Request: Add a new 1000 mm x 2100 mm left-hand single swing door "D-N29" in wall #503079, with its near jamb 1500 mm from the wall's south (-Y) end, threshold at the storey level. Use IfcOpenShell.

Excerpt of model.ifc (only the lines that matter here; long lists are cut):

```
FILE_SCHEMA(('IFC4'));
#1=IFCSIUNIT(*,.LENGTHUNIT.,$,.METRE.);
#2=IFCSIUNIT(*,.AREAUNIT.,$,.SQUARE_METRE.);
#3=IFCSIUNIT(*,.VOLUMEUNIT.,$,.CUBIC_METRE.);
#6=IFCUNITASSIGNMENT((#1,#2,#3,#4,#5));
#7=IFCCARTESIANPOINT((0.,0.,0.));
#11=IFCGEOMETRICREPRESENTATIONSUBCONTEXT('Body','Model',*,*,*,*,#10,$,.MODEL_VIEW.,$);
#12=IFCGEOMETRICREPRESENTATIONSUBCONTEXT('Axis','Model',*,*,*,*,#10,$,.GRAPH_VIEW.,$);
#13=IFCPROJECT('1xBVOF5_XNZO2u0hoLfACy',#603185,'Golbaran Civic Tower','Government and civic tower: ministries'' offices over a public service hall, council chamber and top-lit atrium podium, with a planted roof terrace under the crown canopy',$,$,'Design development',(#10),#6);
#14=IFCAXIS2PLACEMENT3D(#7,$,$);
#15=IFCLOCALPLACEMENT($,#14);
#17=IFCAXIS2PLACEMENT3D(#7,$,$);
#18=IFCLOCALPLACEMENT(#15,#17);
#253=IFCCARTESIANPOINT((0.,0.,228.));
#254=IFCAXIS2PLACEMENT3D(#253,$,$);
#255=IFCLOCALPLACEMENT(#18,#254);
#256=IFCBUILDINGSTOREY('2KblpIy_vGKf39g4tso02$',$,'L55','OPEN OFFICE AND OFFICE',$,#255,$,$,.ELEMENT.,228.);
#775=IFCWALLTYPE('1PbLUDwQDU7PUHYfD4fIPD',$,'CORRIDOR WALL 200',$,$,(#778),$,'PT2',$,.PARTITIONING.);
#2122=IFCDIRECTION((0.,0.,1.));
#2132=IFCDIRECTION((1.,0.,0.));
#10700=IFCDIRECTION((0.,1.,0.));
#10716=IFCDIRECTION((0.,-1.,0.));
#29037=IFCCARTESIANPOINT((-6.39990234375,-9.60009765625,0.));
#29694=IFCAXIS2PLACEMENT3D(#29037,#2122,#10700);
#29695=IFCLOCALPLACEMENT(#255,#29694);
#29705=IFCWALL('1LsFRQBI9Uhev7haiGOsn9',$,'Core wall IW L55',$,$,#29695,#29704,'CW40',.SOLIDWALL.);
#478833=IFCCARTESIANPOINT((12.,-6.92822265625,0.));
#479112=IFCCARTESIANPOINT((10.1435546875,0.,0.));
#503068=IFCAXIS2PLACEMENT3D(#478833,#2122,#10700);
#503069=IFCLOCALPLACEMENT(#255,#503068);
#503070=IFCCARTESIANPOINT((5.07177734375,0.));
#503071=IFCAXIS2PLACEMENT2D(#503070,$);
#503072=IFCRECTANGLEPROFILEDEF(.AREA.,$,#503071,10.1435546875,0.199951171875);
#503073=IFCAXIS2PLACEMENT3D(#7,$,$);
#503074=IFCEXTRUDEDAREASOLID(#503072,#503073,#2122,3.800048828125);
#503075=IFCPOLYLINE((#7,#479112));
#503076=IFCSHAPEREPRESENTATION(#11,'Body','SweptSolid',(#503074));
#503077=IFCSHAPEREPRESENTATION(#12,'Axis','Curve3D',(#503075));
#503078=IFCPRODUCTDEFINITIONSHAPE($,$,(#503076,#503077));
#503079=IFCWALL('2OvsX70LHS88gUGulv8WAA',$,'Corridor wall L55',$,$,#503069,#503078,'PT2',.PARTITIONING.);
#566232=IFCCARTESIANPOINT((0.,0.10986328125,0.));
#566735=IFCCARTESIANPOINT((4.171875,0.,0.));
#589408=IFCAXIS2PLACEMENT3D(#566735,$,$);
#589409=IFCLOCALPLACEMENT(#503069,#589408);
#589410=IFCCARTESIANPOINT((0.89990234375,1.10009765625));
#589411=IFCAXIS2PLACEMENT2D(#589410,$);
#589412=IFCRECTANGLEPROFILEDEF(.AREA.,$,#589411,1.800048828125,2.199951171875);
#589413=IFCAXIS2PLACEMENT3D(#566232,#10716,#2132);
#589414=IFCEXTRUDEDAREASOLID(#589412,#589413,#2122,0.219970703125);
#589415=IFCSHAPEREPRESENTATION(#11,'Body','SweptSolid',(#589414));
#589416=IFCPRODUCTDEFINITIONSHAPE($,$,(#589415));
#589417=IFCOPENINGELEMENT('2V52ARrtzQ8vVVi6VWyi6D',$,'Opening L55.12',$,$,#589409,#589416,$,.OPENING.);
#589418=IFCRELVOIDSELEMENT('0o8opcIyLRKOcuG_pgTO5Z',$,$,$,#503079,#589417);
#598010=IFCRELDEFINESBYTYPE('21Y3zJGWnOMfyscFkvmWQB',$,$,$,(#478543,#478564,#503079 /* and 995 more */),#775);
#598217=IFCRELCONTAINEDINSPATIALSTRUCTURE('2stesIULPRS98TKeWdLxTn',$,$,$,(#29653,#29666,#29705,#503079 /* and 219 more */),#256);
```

```python
import numpy as np
import ifcopenshell
import ifcopenshell.api.feature
import ifcopenshell.api.geometry
import ifcopenshell.api.root
import ifcopenshell.api.spatial
import ifcopenshell.geom
import ifcopenshell.util.element
import ifcopenshell.util.placement
import ifcopenshell.util.representation
import ifcopenshell.util.shape
import ifcopenshell.util.unit

model = ifcopenshell.open("model.ifc")
unit_scale = ifcopenshell.util.unit.calculate_unit_scale(model)
settings = ifcopenshell.geom.settings()


def volume(element):
    """Net volume in cubic metres, openings subtracted."""
    shape = ifcopenshell.geom.create_shape(settings, element)
    return ifcopenshell.util.shape.get_volume(shape.geometry)


wall = model.by_id(503079)
storey = ifcopenshell.util.element.get_container(wall, ifc_class="IfcBuildingStorey")
context = ifcopenshell.util.representation.get_context(model, "Model", "Body", "MODEL_VIEW")
before = volume(wall)

width, height, from_end, sill = 1, 2.1, 1.5, 0.0  # metres

# The wall runs along its own X axis, and the end named is its -X end.
wall_shape = ifcopenshell.geom.create_shape(settings, wall)
x, y, z = ifcopenshell.util.shape.get_vertices(wall_shape.geometry).T
start = x.min() + from_end
face, thickness = float(y.min()), float(y.max() - y.min())
wall_matrix = ifcopenshell.util.placement.get_local_placement(wall.ObjectPlacement)
level = ifcopenshell.util.placement.get_local_placement(storey.ObjectPlacement)[2, 3]


def in_wall(x, y):
    """Placement at x, y metres in the wall's axes, at sill height."""
    matrix = wall_matrix.copy()
    matrix[:, 3] = wall_matrix @ np.array([x / unit_scale, y / unit_scale, 0.0, 1.0])
    matrix[2, 3] = level + sill / unit_scale
    return matrix


# Opening: a box that overshoots both wall faces by 50 mm.
opening = ifcopenshell.api.root.create_entity(model, ifc_class="IfcOpeningElement", predefined_type="OPENING")
box = ifcopenshell.api.geometry.add_wall_representation(
    model, context=context, length=width, height=height, thickness=thickness + 0.1
)
ifcopenshell.api.geometry.assign_representation(model, product=opening, representation=box)
ifcopenshell.api.geometry.edit_object_placement(model, product=opening, matrix=in_wall(start, face - 0.05), is_si=False)
ifcopenshell.api.feature.add_feature(model, feature=opening, element=wall)

door = ifcopenshell.api.root.create_entity(model, ifc_class="IfcDoor", name="D-N29", predefined_type="DOOR")
door.OverallWidth, door.OverallHeight = width / unit_scale, height / unit_scale
door.OperationType = "SINGLE_SWING_LEFT"
body = ifcopenshell.api.geometry.add_door_representation(
    model,
    context=context,
    overall_width=door.OverallWidth,
    overall_height=door.OverallHeight,
    operation_type="SINGLE_SWING_LEFT",
    lining_properties={"LiningDepth": thickness / unit_scale, "ThresholdDepth": thickness / unit_scale},
)
ifcopenshell.api.geometry.assign_representation(model, product=door, representation=body)
ifcopenshell.api.spatial.assign_container(model, products=[door], relating_structure=storey)
ifcopenshell.api.feature.add_filling(model, opening=opening, element=door)

# The lining spans the wall, so the door starts at the wall face.
ifcopenshell.api.geometry.edit_object_placement(model, product=door, matrix=in_wall(start, face), is_si=False)

after = volume(wall)

print(f"wall volume {before:.3f} -> {after:.3f} m3")

model.write("model-out.ifc")
```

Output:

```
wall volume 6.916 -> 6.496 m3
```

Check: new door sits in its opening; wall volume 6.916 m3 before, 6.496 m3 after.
